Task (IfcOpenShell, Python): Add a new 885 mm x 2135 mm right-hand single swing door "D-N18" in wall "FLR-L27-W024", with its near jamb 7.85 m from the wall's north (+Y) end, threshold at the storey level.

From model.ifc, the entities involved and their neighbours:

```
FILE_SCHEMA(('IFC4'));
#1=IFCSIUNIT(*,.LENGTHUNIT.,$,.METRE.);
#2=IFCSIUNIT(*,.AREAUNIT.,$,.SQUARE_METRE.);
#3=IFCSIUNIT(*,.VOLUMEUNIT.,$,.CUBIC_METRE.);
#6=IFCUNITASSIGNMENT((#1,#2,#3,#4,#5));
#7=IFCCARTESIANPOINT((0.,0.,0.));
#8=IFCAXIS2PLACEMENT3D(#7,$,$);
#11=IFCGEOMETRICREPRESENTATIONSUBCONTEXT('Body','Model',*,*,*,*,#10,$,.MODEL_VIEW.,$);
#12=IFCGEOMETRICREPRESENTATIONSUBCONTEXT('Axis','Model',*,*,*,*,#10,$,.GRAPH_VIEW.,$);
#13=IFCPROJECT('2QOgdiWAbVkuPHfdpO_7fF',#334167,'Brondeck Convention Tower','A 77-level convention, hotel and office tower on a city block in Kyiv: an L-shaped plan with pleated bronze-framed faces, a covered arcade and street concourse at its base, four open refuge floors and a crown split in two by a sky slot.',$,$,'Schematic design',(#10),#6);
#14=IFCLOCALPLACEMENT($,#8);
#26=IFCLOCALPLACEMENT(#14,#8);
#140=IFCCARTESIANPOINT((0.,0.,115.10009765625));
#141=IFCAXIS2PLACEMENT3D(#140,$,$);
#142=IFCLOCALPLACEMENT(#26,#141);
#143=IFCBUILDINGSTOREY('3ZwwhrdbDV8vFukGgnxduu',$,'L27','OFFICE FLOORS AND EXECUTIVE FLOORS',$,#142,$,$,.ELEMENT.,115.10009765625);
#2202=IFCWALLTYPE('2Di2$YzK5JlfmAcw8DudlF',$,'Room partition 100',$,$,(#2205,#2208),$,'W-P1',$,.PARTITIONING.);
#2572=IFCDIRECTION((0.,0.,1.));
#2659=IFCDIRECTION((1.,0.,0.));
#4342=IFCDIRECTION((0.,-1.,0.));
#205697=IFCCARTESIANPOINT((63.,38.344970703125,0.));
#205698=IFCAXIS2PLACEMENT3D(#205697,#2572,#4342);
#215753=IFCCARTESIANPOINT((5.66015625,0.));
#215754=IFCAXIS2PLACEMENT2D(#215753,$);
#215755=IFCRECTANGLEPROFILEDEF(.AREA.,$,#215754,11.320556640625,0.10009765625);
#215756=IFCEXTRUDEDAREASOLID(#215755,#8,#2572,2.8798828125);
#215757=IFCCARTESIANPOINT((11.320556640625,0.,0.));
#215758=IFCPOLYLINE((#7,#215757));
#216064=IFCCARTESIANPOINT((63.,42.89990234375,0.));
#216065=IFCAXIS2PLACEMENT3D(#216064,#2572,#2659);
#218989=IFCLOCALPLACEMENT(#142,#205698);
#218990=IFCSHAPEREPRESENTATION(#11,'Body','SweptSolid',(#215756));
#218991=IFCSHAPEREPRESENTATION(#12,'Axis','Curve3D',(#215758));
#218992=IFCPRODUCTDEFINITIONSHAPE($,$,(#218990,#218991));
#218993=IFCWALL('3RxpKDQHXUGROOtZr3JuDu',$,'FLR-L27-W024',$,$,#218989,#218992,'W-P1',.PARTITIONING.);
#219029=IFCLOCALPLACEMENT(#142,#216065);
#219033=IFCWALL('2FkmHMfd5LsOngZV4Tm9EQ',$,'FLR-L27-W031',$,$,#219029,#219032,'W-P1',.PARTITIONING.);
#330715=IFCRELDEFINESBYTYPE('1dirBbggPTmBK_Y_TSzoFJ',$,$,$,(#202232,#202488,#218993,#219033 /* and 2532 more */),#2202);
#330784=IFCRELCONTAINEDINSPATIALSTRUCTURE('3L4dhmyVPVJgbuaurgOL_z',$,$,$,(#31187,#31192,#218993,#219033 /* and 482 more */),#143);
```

```python
import numpy as np
import ifcopenshell
import ifcopenshell.api.feature
import ifcopenshell.api.geometry
import ifcopenshell.api.root
import ifcopenshell.api.spatial
import ifcopenshell.geom
import ifcopenshell.util.element
import ifcopenshell.util.placement
import ifcopenshell.util.representation
import ifcopenshell.util.shape
import ifcopenshell.util.unit

model = ifcopenshell.open("model.ifc")
unit_scale = ifcopenshell.util.unit.calculate_unit_scale(model)
settings = ifcopenshell.geom.settings()


def volume(element):
    """Net volume in cubic metres, openings subtracted."""
    shape = ifcopenshell.geom.create_shape(settings, element)
    return ifcopenshell.util.shape.get_volume(shape.geometry)


wall = model.by_guid("3RxpKDQHXUGROOtZr3JuDu")
storey = ifcopenshell.util.element.get_container(wall, ifc_class="IfcBuildingStorey")
context = ifcopenshell.util.representation.get_context(model, "Model", "Body", "MODEL_VIEW")
before = volume(wall)

width, height, from_end, sill = 0.885, 2.135, 7.85, 0.0  # metres

# The wall runs along its own X axis, and the end named is its -X end.
wall_shape = ifcopenshell.geom.create_shape(settings, wall)
x, y, z = ifcopenshell.util.shape.get_vertices(wall_shape.geometry).T
start = x.min() + from_end
face, thickness = float(y.min()), float(y.max() - y.min())
wall_matrix = ifcopenshell.util.placement.get_local_placement(wall.ObjectPlacement)
level = ifcopenshell.util.placement.get_local_placement(storey.ObjectPlacement)[2, 3]


def in_wall(x, y):
    """Placement at x, y metres in the wall's axes, at sill height."""
    matrix = wall_matrix.copy()
    matrix[:, 3] = wall_matrix @ np.array([x / unit_scale, y / unit_scale, 0.0, 1.0])
    matrix[2, 3] = level + sill / unit_scale
    return matrix


# Opening: a box that overshoots both wall faces by 50 mm.
opening = ifcopenshell.api.root.create_entity(model, ifc_class="IfcOpeningElement", predefined_type="OPENING")
box = ifcopenshell.api.geometry.add_wall_representation(
    model, context=context, length=width, height=height, thickness=thickness + 0.1
)
ifcopenshell.api.geometry.assign_representation(model, product=opening, representation=box)
ifcopenshell.api.geometry.edit_object_placement(model, product=opening, matrix=in_wall(start, face - 0.05), is_si=False)
ifcopenshell.api.feature.add_feature(model, feature=opening, element=wall)

door = ifcopenshell.api.root.create_entity(model, ifc_class="IfcDoor", name="D-N18", predefined_type="DOOR")
door.OverallWidth, door.OverallHeight = width / unit_scale, height / unit_scale
door.OperationType = "SINGLE_SWING_RIGHT"
body = ifcopenshell.api.geometry.add_door_representation(
    model,
    context=context,
    overall_width=door.OverallWidth,
    overall_height=door.OverallHeight,
    operation_type="SINGLE_SWING_RIGHT",
    lining_properties={"LiningDepth": thickness / unit_scale, "ThresholdDepth": thickness / unit_scale},
)
ifcopenshell.api.geometry.assign_representation(model, product=door, representation=body)
ifcopenshell.api.spatial.assign_container(model, products=[door], relating_structure=storey)
ifcopenshell.api.feature.add_filling(model, opening=opening, element=door)

# The lining spans the wall, so the door starts at the wall face.
ifcopenshell.api.geometry.edit_object_placement(model, product=door, matrix=in_wall(start, face), is_si=False)

after = volume(wall)

print(f"wall volume {before:.3f} -> {after:.3f} m3")

model.write("model_v2.ifc")
```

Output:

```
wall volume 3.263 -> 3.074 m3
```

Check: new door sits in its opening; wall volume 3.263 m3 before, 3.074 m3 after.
